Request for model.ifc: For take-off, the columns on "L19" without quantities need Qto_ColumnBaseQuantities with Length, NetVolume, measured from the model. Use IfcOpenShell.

First a look at what the model holds.

```python
import ifcopenshell
import ifcopenshell.util.element
import ifcopenshell.util.unit

model = ifcopenshell.open("model.ifc")
print(model.schema)
for unit_type in ("LENGTHUNIT", "AREAUNIT", "VOLUMEUNIT"):
    print(unit_type, ifcopenshell.util.unit.calculate_unit_scale(model, unit_type))
storey = next(s for s in model.by_type("IfcBuildingStorey") if s.Name == "L19")
columns = [e for e in ifcopenshell.util.element.get_decomposition(storey) if e.is_a("IfcColumn")]
for e in sorted(columns, key=lambda e: e.id()):
    print(e.id(), e.is_a(), e.Name, list(ifcopenshell.util.element.get_psets(e, qtos_only=True)), sep=" | ")
```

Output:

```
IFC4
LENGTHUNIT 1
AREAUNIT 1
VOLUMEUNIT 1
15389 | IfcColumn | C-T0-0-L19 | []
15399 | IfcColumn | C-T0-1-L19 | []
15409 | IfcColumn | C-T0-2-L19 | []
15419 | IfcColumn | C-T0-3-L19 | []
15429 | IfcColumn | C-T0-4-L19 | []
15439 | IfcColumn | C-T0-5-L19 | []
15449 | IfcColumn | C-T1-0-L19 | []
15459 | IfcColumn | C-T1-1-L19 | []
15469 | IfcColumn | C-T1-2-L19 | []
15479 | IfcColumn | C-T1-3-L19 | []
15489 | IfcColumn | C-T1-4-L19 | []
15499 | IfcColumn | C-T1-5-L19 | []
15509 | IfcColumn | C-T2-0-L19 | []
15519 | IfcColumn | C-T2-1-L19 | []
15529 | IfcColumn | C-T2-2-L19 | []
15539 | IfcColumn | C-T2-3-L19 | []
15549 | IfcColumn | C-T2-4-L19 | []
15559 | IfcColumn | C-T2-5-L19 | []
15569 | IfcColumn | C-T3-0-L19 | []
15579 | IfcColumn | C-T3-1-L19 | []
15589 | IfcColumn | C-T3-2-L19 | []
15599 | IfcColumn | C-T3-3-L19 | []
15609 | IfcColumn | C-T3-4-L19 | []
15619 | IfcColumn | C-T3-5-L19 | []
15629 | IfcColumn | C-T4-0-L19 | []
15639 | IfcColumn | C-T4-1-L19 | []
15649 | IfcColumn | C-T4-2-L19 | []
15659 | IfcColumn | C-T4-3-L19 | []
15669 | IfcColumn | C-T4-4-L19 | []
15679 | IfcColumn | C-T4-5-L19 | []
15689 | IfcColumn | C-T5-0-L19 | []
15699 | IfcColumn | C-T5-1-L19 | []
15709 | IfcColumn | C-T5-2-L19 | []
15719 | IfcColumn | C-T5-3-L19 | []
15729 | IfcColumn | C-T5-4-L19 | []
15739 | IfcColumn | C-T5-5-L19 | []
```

```python
import ifcopenshell
import ifcopenshell.api.pset
import ifcopenshell.geom
import ifcopenshell.util.element
import ifcopenshell.util.shape
import ifcopenshell.util.unit

model = ifcopenshell.open("model.ifc")
unit_scale = ifcopenshell.util.unit.calculate_unit_scale(model)
volume_scale = ifcopenshell.util.unit.calculate_unit_scale(model, "VOLUMEUNIT")
settings = ifcopenshell.geom.settings()

storey = next(s for s in model.by_type("IfcBuildingStorey") if s.Name == "L19")
columns = [e for e in ifcopenshell.util.element.get_decomposition(storey) if e.is_a("IfcColumn")]

for e in sorted(columns, key=lambda e: e.id()):
    if ifcopenshell.util.element.get_psets(e, qtos_only=True, should_inherit=False):
        continue
    # Geometry comes back in metres, in the element's own axes.
    shape = ifcopenshell.geom.create_shape(settings, e)
    values = {
        "Length": ifcopenshell.util.shape.get_z(shape.geometry) / unit_scale,
        "NetVolume": ifcopenshell.util.shape.get_volume(shape.geometry) / volume_scale,
    }
    qto = ifcopenshell.api.pset.add_qto(model, product=e, name="Qto_ColumnBaseQuantities")
    ifcopenshell.api.pset.edit_qto(model, qto=qto, properties=values)
    print(e.id(), {k: round(v, 3) for k, v in values.items()})

model.write("model_edited.ifc")
```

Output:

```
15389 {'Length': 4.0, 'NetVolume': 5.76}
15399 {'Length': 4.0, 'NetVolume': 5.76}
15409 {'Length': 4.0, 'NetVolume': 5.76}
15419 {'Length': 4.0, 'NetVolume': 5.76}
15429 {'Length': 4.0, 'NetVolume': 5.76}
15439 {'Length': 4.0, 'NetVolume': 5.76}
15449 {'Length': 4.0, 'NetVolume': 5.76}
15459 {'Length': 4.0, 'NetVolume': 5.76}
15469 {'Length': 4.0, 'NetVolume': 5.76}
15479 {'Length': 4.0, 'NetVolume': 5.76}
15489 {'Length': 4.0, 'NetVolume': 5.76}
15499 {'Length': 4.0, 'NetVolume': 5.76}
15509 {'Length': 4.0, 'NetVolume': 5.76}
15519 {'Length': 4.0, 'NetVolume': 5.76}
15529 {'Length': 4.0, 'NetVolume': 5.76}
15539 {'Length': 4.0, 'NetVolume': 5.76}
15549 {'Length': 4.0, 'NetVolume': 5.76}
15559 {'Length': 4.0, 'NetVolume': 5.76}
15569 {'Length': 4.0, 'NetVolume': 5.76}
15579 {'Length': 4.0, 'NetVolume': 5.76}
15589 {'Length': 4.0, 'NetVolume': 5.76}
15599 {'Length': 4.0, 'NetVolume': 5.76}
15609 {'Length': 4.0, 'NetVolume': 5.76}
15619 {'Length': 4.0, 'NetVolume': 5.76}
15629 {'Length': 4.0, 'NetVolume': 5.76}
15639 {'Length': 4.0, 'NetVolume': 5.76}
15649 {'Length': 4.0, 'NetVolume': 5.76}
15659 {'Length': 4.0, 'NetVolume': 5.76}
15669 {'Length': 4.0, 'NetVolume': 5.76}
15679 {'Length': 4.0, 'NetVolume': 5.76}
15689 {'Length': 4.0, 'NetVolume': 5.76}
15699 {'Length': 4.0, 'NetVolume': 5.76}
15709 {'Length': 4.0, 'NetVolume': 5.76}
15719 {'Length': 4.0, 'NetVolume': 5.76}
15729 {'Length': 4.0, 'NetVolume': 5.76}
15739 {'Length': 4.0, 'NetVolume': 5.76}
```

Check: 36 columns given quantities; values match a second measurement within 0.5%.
